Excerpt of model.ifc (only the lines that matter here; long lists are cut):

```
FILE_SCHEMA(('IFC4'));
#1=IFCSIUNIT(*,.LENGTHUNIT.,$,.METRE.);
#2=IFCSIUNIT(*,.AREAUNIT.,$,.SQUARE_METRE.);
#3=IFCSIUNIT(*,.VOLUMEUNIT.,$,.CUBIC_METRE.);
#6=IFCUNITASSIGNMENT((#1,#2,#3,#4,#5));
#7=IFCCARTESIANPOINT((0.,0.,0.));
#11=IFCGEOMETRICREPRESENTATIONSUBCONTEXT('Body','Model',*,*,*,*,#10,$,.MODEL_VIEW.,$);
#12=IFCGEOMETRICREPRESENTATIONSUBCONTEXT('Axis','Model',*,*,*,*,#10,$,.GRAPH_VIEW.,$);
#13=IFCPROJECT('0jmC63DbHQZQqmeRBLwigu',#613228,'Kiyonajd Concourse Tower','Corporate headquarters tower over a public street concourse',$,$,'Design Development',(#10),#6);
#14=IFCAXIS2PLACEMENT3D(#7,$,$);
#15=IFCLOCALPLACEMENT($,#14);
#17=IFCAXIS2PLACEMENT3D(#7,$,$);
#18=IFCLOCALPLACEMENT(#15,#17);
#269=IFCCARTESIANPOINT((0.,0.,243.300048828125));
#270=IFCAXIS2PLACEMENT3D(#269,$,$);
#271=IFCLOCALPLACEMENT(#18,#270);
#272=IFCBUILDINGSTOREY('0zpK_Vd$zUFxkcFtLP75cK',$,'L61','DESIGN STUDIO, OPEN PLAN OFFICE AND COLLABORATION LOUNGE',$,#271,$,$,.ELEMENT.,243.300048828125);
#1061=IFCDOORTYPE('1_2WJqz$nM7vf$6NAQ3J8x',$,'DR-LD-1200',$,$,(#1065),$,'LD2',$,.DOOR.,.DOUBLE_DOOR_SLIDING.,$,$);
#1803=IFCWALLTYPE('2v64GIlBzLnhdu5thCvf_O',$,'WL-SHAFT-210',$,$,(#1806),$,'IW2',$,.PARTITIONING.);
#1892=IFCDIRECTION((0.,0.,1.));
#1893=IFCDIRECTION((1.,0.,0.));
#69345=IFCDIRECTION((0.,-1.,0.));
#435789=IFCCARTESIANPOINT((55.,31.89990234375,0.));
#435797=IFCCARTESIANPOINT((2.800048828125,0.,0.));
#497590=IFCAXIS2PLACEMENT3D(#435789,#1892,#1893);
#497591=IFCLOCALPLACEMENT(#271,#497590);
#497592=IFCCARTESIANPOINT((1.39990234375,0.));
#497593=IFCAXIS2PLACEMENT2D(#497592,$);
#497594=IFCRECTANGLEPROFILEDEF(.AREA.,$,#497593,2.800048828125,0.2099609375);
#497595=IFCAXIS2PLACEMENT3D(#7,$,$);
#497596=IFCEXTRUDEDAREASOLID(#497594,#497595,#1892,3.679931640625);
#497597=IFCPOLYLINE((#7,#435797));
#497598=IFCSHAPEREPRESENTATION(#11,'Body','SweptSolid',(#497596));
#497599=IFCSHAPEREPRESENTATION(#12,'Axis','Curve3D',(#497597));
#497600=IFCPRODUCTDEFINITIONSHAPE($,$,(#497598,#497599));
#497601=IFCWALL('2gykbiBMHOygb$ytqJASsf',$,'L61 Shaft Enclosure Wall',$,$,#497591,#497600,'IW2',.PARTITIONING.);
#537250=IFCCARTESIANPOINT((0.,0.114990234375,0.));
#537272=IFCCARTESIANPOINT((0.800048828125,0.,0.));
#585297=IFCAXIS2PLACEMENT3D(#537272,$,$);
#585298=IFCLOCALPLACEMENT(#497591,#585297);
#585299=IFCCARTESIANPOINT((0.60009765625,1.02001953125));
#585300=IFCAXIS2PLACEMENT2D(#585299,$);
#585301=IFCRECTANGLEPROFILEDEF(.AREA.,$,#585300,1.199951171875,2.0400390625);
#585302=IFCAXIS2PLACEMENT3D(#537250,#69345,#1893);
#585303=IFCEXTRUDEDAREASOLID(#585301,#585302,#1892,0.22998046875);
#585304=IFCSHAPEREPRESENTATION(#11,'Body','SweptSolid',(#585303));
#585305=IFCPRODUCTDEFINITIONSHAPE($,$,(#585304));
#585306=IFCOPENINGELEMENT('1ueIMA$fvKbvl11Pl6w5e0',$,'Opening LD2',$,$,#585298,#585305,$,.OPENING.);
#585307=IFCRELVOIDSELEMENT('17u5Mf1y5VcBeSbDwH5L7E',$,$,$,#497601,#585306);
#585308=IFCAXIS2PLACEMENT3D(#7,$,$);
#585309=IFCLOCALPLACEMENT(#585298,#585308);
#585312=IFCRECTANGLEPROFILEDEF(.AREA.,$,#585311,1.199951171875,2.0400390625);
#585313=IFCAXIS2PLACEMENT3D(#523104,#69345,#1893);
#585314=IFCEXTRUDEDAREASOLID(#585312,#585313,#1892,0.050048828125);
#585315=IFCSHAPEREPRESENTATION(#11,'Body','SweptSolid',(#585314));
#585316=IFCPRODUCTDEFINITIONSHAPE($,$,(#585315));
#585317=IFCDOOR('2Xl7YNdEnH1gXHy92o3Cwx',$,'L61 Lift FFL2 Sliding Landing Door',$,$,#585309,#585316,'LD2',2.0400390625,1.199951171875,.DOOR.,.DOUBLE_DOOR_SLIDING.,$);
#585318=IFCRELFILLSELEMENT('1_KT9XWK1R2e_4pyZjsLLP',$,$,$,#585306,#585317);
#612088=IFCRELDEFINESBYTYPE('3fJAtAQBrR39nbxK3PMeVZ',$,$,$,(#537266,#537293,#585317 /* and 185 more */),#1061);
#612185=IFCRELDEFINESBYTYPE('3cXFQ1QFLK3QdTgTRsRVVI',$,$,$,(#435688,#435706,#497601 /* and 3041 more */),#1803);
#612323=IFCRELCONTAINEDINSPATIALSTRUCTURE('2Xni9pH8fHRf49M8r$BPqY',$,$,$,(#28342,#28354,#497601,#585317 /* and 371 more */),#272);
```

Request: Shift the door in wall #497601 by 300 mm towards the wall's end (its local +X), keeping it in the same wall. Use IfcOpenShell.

```python
import ifcopenshell
import ifcopenshell.api.geometry
import ifcopenshell.util.placement
import ifcopenshell.util.unit

model = ifcopenshell.open("model.ifc")
unit_scale = ifcopenshell.util.unit.calculate_unit_scale(model)

door = model.by_guid("2Xl7YNdEnH1gXHy92o3Cwx")
opening = door.FillsVoids[0].RelatingOpeningElement
wall = opening.VoidsElements[0].RelatingBuildingElement

wall_matrix = ifcopenshell.util.placement.get_local_placement(wall.ObjectPlacement)
shift = wall_matrix[:3, 0] * 0.3 / unit_scale
before = ifcopenshell.util.placement.get_local_placement(door.ObjectPlacement)[:3, 3].copy()

# The door is placed relative to its opening, so it follows when the opening moves.
matrix = ifcopenshell.util.placement.get_local_placement(opening.ObjectPlacement)
matrix[:3, 3] += shift
ifcopenshell.api.geometry.edit_object_placement(
    model, product=opening, matrix=matrix, is_si=False, should_transform_children=True
)

after = ifcopenshell.util.placement.get_local_placement(door.ObjectPlacement)[:3, 3]
print("door moved by", (after - before).round(3) + 0.0)

model.write("model_rev.ifc")
```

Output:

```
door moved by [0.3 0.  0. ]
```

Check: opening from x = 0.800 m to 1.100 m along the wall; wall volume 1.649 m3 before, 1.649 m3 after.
